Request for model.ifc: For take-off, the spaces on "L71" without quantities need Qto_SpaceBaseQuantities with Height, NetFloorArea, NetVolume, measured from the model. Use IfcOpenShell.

First a look at what the model holds.

```python
import ifcopenshell
import ifcopenshell.util.element
import ifcopenshell.util.unit

model = ifcopenshell.open("model.ifc")
print(model.schema)
for unit_type in ("LENGTHUNIT", "AREAUNIT", "VOLUMEUNIT"):
    print(unit_type, ifcopenshell.util.unit.calculate_unit_scale(model, unit_type))
storey = next(s for s in model.by_type("IfcBuildingStorey") if s.Name == "L71")
spaces = [e for e in ifcopenshell.util.element.get_decomposition(storey) if e.is_a("IfcSpace")]
for e in sorted(spaces, key=lambda e: e.id()):
    print(e.id(), e.is_a(), e.Name, list(ifcopenshell.util.element.get_psets(e, qtos_only=True)), sep=" | ")
```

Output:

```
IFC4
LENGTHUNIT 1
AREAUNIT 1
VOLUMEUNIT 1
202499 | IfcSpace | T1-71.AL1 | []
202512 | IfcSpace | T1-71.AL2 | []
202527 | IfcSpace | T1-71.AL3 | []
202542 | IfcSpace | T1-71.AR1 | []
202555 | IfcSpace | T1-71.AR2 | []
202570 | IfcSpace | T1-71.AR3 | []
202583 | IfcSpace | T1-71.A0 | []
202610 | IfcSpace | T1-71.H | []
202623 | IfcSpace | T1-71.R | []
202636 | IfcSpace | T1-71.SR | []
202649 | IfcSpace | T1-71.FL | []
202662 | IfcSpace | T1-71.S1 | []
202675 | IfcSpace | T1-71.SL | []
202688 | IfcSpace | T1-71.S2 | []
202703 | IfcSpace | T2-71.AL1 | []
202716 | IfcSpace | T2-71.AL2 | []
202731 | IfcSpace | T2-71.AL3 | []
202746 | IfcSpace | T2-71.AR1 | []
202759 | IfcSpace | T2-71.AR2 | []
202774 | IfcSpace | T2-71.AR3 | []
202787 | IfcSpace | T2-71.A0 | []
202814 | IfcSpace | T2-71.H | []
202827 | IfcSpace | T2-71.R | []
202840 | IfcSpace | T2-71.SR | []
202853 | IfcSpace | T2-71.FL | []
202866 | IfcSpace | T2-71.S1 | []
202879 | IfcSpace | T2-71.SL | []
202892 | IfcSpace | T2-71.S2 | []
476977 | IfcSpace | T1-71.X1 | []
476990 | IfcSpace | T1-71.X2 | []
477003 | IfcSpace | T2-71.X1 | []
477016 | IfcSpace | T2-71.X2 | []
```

```python
import ifcopenshell
import ifcopenshell.api.pset
import ifcopenshell.geom
import ifcopenshell.util.element
import ifcopenshell.util.shape
import ifcopenshell.util.unit

model = ifcopenshell.open("model.ifc")
unit_scale = ifcopenshell.util.unit.calculate_unit_scale(model)
area_scale = ifcopenshell.util.unit.calculate_unit_scale(model, "AREAUNIT")
volume_scale = ifcopenshell.util.unit.calculate_unit_scale(model, "VOLUMEUNIT")
settings = ifcopenshell.geom.settings()

storey = next(s for s in model.by_type("IfcBuildingStorey") if s.Name == "L71")
spaces = [e for e in ifcopenshell.util.element.get_decomposition(storey) if e.is_a("IfcSpace")]

for e in sorted(spaces, key=lambda e: e.id()):
    if ifcopenshell.util.element.get_psets(e, qtos_only=True, should_inherit=False):
        continue
    # Geometry comes back in metres, in the element's own axes.
    shape = ifcopenshell.geom.create_shape(settings, e)
    values = {
        "Height": ifcopenshell.util.shape.get_z(shape.geometry) / unit_scale,
        "NetFloorArea": ifcopenshell.util.shape.get_footprint_area(shape.geometry) / area_scale,
        "NetVolume": ifcopenshell.util.shape.get_volume(shape.geometry) / volume_scale,
    }
    qto = ifcopenshell.api.pset.add_qto(model, product=e, name="Qto_SpaceBaseQuantities")
    ifcopenshell.api.pset.edit_qto(model, qto=qto, properties=values)
    print(e.id(), {k: round(v, 3) for k, v in values.items()})

model.write("model_v2.ifc")
```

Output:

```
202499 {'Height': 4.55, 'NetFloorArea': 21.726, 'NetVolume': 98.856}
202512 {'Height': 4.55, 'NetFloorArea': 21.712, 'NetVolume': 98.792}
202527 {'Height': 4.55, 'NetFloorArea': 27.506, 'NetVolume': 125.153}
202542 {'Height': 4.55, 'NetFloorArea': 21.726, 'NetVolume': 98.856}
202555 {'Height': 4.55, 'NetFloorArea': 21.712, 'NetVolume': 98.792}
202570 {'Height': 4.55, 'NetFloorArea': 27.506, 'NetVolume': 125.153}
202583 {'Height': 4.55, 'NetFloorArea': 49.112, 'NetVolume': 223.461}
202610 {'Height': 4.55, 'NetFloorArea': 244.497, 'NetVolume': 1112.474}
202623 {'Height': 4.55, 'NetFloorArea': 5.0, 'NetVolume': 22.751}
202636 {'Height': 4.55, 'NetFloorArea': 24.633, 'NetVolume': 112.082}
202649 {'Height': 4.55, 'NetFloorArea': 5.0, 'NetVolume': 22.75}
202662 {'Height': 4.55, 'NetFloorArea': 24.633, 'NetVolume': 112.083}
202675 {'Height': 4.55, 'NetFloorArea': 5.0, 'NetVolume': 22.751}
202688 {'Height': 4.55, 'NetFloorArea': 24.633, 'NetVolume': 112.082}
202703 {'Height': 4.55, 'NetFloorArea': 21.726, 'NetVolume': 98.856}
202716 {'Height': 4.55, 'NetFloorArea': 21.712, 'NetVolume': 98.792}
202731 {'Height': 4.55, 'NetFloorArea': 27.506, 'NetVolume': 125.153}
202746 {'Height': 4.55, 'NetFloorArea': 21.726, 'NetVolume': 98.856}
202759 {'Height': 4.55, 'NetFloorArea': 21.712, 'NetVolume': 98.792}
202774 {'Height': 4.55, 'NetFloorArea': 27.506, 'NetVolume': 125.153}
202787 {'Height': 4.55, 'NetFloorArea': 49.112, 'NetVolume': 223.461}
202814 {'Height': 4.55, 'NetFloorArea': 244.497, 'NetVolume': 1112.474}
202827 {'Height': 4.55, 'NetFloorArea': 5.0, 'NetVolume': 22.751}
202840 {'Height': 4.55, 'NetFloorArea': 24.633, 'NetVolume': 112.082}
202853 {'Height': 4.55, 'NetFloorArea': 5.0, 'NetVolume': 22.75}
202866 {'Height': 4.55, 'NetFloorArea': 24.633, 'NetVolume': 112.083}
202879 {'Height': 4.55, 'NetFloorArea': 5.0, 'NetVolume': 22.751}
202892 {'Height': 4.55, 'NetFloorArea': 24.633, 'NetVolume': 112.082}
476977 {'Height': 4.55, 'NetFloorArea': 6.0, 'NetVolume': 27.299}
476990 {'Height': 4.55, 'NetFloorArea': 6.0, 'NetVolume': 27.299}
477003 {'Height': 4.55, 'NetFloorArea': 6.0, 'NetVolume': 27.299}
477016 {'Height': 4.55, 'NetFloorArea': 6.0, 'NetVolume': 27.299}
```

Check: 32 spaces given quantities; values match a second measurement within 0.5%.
